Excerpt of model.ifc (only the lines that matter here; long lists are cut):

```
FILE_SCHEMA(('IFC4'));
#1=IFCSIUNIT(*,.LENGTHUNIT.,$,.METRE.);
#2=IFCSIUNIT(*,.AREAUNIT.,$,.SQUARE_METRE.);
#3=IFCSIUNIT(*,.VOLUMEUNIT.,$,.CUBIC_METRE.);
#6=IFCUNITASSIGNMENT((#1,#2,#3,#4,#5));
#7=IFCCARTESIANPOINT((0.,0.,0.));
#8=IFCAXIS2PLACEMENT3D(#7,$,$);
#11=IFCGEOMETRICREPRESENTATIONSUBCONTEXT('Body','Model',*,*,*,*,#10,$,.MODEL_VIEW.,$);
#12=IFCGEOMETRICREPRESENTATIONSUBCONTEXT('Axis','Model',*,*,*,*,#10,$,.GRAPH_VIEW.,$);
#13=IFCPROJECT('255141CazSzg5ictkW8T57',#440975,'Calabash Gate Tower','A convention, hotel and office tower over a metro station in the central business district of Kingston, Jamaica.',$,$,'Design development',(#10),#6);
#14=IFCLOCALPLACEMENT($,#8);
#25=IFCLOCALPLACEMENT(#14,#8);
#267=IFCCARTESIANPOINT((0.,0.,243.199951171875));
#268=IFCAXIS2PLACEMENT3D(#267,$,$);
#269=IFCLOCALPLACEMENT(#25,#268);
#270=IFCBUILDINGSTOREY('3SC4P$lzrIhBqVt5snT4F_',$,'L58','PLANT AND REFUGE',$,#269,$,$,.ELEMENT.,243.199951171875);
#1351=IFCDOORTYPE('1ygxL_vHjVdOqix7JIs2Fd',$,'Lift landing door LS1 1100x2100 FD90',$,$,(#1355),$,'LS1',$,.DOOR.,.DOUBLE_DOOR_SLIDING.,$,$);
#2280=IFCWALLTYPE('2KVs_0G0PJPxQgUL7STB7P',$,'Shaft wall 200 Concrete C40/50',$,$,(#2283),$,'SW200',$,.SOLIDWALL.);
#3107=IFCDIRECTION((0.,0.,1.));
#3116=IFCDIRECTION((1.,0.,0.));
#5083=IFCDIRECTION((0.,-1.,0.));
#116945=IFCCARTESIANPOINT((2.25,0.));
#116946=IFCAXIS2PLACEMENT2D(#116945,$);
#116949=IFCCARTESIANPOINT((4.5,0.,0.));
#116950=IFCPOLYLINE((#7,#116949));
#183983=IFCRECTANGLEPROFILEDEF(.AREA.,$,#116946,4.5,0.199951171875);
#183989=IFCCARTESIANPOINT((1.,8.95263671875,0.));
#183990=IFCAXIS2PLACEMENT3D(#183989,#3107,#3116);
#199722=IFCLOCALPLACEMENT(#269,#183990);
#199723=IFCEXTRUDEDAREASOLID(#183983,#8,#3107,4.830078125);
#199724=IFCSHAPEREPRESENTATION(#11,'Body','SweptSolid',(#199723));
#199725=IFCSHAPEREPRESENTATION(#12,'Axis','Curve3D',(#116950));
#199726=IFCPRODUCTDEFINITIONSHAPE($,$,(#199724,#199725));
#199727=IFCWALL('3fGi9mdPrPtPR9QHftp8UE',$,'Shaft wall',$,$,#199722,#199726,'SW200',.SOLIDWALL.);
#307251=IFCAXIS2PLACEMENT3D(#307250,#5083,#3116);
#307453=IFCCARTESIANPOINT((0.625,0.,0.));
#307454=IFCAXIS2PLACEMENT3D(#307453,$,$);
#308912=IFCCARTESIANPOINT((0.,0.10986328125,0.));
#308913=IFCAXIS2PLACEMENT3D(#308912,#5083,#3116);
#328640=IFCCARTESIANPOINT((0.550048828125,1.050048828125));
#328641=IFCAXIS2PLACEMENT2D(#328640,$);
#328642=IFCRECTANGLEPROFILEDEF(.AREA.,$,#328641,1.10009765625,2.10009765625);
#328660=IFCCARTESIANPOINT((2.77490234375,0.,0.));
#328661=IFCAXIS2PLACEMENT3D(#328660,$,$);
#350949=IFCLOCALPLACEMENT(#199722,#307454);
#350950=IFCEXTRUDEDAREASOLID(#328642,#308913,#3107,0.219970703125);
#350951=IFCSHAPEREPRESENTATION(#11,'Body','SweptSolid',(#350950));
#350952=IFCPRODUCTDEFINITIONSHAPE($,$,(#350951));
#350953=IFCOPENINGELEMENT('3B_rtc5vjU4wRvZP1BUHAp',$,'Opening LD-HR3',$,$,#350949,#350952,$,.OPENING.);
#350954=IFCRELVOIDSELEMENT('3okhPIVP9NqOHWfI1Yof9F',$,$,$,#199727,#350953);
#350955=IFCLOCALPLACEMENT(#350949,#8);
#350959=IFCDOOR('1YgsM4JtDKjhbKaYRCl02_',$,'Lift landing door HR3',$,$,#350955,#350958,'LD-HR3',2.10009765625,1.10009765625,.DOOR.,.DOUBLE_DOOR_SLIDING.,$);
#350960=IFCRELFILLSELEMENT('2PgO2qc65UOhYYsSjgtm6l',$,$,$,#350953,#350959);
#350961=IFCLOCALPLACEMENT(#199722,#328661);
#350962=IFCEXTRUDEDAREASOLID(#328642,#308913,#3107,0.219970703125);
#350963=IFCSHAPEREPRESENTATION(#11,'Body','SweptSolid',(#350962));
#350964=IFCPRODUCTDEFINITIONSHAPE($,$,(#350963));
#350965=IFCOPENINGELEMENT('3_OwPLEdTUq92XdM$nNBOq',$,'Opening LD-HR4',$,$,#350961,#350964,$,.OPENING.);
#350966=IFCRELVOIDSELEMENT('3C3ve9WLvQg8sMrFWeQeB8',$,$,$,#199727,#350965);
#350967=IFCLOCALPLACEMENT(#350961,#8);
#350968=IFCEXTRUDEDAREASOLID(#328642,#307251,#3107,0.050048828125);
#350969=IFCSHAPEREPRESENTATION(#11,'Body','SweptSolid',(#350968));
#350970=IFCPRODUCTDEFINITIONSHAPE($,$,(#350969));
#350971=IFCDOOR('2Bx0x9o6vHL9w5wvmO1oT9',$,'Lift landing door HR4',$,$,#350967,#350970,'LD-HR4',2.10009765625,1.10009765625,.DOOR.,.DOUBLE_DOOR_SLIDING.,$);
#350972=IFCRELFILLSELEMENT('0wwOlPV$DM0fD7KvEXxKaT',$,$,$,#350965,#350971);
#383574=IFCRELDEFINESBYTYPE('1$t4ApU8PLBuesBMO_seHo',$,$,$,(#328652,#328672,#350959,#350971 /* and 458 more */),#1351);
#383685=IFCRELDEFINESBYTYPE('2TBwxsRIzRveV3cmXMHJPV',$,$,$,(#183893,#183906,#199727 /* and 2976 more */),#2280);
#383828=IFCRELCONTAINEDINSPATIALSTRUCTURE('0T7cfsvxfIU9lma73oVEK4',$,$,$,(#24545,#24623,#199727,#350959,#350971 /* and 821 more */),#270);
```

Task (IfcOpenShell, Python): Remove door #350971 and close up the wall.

```python
import ifcopenshell
import ifcopenshell.api.feature
import ifcopenshell.api.root
import ifcopenshell.geom
import ifcopenshell.util.shape

model = ifcopenshell.open("model.ifc")
settings = ifcopenshell.geom.settings()


def volume(element):
    """Net volume in cubic metres, openings subtracted."""
    shape = ifcopenshell.geom.create_shape(settings, element)
    return ifcopenshell.util.shape.get_volume(shape.geometry)


door = model.by_guid("2Bx0x9o6vHL9w5wvmO1oT9")
opening = door.FillsVoids[0].RelatingOpeningElement
wall = opening.VoidsElements[0].RelatingBuildingElement
before = volume(wall)

ifcopenshell.api.root.remove_product(model, product=door)
ifcopenshell.api.feature.remove_feature(model, feature=opening)

after = volume(wall)

print(f"wall volume {before:.3f} -> {after:.3f} m3")

model.write("model_updated.ifc")
```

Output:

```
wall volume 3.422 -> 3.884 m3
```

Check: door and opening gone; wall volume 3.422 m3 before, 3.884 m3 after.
